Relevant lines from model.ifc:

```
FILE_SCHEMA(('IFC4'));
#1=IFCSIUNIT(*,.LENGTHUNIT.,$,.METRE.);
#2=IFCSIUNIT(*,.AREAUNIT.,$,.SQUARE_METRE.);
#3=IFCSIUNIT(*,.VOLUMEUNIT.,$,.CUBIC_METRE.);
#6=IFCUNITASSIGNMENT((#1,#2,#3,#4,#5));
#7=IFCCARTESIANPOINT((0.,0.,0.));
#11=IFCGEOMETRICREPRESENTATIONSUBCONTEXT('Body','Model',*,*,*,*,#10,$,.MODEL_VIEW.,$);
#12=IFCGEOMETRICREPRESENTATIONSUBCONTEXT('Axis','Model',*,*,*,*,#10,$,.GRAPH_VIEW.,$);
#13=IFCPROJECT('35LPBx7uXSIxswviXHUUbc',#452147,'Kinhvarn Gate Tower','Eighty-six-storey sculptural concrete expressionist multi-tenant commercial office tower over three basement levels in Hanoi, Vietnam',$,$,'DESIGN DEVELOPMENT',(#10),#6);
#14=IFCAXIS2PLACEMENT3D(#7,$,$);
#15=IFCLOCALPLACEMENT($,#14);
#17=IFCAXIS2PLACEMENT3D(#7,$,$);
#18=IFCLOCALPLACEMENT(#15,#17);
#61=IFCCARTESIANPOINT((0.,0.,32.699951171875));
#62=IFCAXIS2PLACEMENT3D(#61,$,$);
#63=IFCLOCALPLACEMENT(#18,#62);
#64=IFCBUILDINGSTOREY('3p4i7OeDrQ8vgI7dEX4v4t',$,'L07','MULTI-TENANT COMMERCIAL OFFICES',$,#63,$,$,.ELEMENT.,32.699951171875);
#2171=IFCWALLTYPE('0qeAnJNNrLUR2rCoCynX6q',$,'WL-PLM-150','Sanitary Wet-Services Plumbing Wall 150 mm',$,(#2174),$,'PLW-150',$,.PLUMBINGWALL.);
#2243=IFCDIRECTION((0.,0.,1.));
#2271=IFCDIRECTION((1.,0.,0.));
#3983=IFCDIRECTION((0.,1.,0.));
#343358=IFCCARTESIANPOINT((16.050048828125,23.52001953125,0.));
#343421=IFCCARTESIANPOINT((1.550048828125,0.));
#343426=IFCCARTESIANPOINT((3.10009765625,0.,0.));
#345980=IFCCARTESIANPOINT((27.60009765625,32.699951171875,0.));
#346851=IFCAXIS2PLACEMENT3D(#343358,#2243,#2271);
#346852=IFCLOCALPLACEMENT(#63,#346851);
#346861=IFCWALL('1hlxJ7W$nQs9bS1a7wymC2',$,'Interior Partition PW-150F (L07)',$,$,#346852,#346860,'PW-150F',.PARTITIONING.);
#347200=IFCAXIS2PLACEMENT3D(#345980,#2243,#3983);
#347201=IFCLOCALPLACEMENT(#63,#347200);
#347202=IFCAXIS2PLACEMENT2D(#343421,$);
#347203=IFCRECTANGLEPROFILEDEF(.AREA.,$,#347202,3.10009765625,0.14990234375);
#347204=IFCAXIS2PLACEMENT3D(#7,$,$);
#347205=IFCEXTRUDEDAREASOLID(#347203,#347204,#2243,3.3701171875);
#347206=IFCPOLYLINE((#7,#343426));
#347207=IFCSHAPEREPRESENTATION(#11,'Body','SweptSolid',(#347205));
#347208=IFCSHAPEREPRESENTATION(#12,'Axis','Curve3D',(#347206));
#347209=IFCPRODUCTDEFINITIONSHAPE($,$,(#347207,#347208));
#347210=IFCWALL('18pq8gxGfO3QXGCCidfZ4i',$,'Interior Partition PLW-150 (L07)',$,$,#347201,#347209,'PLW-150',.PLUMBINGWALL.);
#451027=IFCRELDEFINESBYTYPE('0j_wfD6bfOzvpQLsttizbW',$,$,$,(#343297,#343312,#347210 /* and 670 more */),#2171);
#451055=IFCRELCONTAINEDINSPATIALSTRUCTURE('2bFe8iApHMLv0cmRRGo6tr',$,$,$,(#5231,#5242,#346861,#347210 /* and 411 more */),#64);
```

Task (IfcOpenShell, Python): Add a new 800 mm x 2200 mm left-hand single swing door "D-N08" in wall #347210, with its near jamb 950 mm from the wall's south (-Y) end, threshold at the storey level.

```python
import numpy as np
import ifcopenshell
import ifcopenshell.api.feature
import ifcopenshell.api.geometry
import ifcopenshell.api.root
import ifcopenshell.api.spatial
import ifcopenshell.geom
import ifcopenshell.util.element
import ifcopenshell.util.placement
import ifcopenshell.util.representation
import ifcopenshell.util.shape
import ifcopenshell.util.unit

model = ifcopenshell.open("model.ifc")
unit_scale = ifcopenshell.util.unit.calculate_unit_scale(model)
settings = ifcopenshell.geom.settings()


def volume(element):
    """Net volume in cubic metres, openings subtracted."""
    shape = ifcopenshell.geom.create_shape(settings, element)
    return ifcopenshell.util.shape.get_volume(shape.geometry)


wall = model.by_guid("18pq8gxGfO3QXGCCidfZ4i")
storey = ifcopenshell.util.element.get_container(wall, ifc_class="IfcBuildingStorey")
context = ifcopenshell.util.representation.get_context(model, "Model", "Body", "MODEL_VIEW")
before = volume(wall)

width, height, from_end, sill = 0.8, 2.2, 0.95, 0.0  # metres

# The wall runs along its own X axis, and the end named is its -X end.
wall_shape = ifcopenshell.geom.create_shape(settings, wall)
x, y, z = ifcopenshell.util.shape.get_vertices(wall_shape.geometry).T
start = x.min() + from_end
face, thickness = float(y.min()), float(y.max() - y.min())
wall_matrix = ifcopenshell.util.placement.get_local_placement(wall.ObjectPlacement)
level = ifcopenshell.util.placement.get_local_placement(storey.ObjectPlacement)[2, 3]


def in_wall(x, y):
    """Placement at x, y metres in the wall's axes, at sill height."""
    matrix = wall_matrix.copy()
    matrix[:, 3] = wall_matrix @ np.array([x / unit_scale, y / unit_scale, 0.0, 1.0])
    matrix[2, 3] = level + sill / unit_scale
    return matrix


# Opening: a box that overshoots both wall faces by 50 mm.
opening = ifcopenshell.api.root.create_entity(model, ifc_class="IfcOpeningElement", predefined_type="OPENING")
box = ifcopenshell.api.geometry.add_wall_representation(
    model, context=context, length=width, height=height, thickness=thickness + 0.1
)
ifcopenshell.api.geometry.assign_representation(model, product=opening, representation=box)
ifcopenshell.api.geometry.edit_object_placement(model, product=opening, matrix=in_wall(start, face - 0.05), is_si=False)
ifcopenshell.api.feature.add_feature(model, feature=opening, element=wall)

door = ifcopenshell.api.root.create_entity(model, ifc_class="IfcDoor", name="D-N08", predefined_type="DOOR")
door.OverallWidth, door.OverallHeight = width / unit_scale, height / unit_scale
door.OperationType = "SINGLE_SWING_LEFT"
body = ifcopenshell.api.geometry.add_door_representation(
    model,
    context=context,
    overall_width=door.OverallWidth,
    overall_height=door.OverallHeight,
    operation_type="SINGLE_SWING_LEFT",
    lining_properties={"LiningDepth": thickness / unit_scale, "ThresholdDepth": thickness / unit_scale},
)
ifcopenshell.api.geometry.assign_representation(model, product=door, representation=body)
ifcopenshell.api.spatial.assign_container(model, products=[door], relating_structure=storey)
ifcopenshell.api.feature.add_filling(model, opening=opening, element=door)

# The lining spans the wall, so the door starts at the wall face.
ifcopenshell.api.geometry.edit_object_placement(model, product=door, matrix=in_wall(start, face), is_si=False)

after = volume(wall)

print(f"wall volume {before:.3f} -> {after:.3f} m3")

model.write("model-out.ifc")
```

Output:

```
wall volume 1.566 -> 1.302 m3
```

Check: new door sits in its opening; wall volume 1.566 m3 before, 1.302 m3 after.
